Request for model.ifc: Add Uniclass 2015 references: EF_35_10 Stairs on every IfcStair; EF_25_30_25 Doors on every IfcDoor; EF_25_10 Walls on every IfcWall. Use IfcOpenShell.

First a look at what the model holds.

```python
import ifcopenshell

model = ifcopenshell.open("model.ifc")
print(model.schema)
print("classifications:", [c.Name for c in model.by_type("IfcClassification")])
for ifc_class in ("IfcDoor", "IfcRoof", "IfcStair", "IfcWall", "IfcWindow"):
    print(ifc_class, len(model.by_type(ifc_class)))
```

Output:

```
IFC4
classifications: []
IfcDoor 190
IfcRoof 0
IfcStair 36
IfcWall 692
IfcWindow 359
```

```python
import ifcopenshell
import ifcopenshell.api.classification

model = ifcopenshell.open("model.ifc")

system = ifcopenshell.api.classification.add_classification(model, classification="Uniclass 2015")

codes = {
    "IfcStair": ("EF_35_10", "Stairs"),
    "IfcDoor": ("EF_25_30_25", "Doors"),
    "IfcWall": ("EF_25_10", "Walls"),
}
for ifc_class, (code, name) in codes.items():
    products = model.by_type(ifc_class)
    ifcopenshell.api.classification.add_reference(
        model, products=products, classification=system, identification=code, name=name
    )
    print(code, len(products))

model.write("model_edited.ifc")
```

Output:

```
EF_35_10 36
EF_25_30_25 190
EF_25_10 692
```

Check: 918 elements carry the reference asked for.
